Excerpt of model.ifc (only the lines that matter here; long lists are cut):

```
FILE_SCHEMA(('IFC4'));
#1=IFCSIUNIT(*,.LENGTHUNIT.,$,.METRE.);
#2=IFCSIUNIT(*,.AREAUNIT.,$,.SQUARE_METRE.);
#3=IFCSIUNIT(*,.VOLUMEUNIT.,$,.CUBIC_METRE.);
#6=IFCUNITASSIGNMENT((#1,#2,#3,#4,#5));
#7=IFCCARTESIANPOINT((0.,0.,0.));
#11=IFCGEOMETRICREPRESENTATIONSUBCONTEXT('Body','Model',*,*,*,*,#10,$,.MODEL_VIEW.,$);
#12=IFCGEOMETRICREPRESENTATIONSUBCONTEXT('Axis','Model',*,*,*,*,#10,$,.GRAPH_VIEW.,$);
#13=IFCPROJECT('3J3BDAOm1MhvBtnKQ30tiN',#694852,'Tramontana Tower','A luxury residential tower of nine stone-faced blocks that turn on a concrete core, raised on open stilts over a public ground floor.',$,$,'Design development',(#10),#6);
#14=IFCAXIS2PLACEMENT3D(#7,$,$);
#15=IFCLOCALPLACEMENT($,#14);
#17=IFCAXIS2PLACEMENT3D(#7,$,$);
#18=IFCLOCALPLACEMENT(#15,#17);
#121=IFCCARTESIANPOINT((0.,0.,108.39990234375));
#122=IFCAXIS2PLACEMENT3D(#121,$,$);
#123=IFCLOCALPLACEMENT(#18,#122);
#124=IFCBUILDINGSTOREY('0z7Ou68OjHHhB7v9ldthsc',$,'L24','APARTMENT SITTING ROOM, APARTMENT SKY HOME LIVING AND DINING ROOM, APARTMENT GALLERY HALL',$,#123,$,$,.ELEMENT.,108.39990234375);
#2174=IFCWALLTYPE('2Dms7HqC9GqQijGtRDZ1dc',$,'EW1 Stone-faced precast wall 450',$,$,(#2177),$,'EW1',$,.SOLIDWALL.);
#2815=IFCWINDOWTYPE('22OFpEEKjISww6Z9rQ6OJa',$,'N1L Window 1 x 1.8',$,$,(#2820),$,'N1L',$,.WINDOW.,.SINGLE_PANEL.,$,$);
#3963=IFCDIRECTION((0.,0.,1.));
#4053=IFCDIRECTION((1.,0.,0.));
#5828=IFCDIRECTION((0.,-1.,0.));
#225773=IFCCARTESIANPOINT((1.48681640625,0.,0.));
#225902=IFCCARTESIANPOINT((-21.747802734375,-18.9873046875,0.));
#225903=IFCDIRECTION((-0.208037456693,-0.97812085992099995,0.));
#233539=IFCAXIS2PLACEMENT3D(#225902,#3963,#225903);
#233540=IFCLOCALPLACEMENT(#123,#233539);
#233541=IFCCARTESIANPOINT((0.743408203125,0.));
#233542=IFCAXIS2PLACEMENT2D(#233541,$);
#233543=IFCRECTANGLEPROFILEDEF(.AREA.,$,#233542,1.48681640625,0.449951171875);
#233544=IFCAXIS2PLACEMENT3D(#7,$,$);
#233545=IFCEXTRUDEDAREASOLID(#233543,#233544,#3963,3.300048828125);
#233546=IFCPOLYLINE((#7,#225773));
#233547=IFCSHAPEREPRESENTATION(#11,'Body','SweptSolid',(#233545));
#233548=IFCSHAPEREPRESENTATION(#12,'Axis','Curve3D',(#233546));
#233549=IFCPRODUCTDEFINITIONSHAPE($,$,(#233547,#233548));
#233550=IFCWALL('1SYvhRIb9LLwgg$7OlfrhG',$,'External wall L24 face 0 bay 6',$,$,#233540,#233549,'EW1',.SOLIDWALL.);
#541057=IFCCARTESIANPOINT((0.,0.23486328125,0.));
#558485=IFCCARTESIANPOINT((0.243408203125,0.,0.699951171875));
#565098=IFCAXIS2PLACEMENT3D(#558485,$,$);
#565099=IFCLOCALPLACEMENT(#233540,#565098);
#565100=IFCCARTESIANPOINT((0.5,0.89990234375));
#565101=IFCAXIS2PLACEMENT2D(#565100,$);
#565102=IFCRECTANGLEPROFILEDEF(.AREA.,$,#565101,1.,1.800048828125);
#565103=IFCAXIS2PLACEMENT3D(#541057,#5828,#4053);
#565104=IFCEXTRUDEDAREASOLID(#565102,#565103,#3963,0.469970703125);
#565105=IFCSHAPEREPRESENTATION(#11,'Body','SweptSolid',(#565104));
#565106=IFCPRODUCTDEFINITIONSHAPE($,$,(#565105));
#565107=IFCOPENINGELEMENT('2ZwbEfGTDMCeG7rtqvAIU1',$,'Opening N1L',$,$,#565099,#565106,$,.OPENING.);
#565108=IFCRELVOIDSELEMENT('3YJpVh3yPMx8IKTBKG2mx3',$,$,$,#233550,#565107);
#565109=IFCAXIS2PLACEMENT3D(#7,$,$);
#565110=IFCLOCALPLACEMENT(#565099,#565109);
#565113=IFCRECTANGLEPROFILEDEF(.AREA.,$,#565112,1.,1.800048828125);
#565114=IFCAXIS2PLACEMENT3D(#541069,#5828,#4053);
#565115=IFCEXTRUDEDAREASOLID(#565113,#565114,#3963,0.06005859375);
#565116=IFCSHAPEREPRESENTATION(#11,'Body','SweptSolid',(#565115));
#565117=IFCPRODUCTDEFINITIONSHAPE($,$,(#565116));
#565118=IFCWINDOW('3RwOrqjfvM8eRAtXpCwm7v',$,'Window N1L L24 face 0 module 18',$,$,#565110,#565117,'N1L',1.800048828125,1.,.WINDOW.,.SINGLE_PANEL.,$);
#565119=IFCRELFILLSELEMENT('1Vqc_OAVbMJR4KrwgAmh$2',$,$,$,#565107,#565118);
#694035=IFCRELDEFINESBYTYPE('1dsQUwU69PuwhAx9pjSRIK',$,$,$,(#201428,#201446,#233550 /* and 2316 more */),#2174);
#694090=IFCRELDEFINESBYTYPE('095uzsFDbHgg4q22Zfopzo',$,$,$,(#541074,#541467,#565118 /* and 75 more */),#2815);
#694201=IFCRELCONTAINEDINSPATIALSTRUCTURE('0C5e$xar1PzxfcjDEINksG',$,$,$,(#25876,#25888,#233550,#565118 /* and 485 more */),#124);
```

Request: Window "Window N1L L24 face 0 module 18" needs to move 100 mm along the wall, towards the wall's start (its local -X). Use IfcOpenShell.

```python
import ifcopenshell
import ifcopenshell.api.geometry
import ifcopenshell.util.placement
import ifcopenshell.util.unit

model = ifcopenshell.open("model.ifc")
unit_scale = ifcopenshell.util.unit.calculate_unit_scale(model)

window = model.by_guid("3RwOrqjfvM8eRAtXpCwm7v")
opening = window.FillsVoids[0].RelatingOpeningElement
wall = opening.VoidsElements[0].RelatingBuildingElement

wall_matrix = ifcopenshell.util.placement.get_local_placement(wall.ObjectPlacement)
shift = wall_matrix[:3, 0] * -0.1 / unit_scale
before = ifcopenshell.util.placement.get_local_placement(window.ObjectPlacement)[:3, 3].copy()

# The window is placed relative to its opening, so it follows when the opening moves.
matrix = ifcopenshell.util.placement.get_local_placement(opening.ObjectPlacement)
matrix[:3, 3] += shift
ifcopenshell.api.geometry.edit_object_placement(
    model, product=opening, matrix=matrix, is_si=False, should_transform_children=True
)

after = ifcopenshell.util.placement.get_local_placement(window.ObjectPlacement)[:3, 3]
print("window moved by", (after - before).round(3) + 0.0)

model.write("model_v2.ifc")
```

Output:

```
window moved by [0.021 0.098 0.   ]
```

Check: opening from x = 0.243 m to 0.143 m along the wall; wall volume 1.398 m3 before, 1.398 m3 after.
